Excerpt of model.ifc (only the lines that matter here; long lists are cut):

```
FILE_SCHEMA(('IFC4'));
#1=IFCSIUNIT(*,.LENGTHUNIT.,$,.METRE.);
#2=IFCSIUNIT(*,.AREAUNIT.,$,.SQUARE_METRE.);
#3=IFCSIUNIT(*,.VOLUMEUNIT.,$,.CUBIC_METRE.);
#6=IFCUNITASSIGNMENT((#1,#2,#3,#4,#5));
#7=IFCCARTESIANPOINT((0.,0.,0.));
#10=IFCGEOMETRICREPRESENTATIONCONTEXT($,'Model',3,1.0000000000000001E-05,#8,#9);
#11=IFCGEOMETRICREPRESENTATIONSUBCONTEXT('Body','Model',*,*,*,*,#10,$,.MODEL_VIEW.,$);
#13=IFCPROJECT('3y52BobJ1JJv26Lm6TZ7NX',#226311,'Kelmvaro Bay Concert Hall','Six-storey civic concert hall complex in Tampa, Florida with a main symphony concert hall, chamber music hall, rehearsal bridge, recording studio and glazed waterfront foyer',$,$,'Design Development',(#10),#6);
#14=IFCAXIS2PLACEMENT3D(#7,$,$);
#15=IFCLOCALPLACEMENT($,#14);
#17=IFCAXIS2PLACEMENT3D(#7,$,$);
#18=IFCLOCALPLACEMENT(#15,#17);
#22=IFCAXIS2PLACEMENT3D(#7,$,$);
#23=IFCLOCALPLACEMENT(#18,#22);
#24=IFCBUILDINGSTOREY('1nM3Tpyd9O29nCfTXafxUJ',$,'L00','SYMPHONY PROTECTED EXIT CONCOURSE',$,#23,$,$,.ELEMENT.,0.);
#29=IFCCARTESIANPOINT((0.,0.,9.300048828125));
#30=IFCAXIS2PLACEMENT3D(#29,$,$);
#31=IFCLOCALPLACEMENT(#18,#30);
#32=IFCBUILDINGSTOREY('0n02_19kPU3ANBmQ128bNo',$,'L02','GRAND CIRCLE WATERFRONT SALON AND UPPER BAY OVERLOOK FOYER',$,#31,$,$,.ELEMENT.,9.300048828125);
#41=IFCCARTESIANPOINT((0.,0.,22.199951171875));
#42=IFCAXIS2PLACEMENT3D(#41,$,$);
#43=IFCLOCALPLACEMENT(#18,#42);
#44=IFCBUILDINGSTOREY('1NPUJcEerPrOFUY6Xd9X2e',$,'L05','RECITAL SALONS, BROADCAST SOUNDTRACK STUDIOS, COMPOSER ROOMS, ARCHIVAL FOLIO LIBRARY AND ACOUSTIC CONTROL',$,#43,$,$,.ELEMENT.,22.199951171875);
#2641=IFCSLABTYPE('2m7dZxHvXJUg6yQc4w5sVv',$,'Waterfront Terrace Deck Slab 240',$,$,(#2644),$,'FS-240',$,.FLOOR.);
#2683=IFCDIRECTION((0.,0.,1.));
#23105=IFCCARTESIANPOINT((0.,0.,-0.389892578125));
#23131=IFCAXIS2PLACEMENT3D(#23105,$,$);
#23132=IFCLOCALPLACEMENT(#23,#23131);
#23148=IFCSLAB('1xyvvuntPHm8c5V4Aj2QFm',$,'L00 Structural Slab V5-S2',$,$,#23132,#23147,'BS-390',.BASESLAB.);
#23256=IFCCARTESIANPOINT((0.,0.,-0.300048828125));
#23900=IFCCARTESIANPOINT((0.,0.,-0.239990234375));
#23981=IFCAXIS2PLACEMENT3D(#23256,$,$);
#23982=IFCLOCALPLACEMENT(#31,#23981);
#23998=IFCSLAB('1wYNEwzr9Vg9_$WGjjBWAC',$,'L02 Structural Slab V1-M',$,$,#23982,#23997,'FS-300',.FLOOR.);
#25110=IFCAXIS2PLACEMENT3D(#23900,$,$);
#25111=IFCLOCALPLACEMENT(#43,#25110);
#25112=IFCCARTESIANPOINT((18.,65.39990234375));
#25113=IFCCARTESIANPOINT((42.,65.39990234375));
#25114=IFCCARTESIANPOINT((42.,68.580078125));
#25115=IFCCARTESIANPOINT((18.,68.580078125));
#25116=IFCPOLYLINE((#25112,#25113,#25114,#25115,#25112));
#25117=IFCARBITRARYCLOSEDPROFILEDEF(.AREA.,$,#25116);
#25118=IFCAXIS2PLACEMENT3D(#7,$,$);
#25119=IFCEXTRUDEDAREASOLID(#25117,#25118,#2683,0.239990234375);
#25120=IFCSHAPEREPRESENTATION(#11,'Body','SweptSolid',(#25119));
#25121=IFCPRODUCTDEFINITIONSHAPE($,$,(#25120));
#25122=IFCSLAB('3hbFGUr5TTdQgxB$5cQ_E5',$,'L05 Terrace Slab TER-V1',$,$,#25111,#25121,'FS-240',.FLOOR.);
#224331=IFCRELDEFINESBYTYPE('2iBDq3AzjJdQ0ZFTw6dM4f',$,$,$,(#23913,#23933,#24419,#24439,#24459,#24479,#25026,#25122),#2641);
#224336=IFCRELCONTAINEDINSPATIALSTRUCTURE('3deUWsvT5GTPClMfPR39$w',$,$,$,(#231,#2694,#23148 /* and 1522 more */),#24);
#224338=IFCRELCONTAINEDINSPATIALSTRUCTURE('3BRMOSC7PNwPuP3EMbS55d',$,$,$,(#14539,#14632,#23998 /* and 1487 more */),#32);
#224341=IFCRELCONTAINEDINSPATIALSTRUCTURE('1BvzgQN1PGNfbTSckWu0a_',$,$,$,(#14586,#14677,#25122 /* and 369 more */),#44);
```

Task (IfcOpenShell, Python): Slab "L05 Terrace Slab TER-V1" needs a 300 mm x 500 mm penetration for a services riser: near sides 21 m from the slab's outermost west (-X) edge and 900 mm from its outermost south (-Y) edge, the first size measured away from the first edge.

```python
import numpy as np
import ifcopenshell
import ifcopenshell.api.feature
import ifcopenshell.api.geometry
import ifcopenshell.api.root
import ifcopenshell.geom
import ifcopenshell.util.placement
import ifcopenshell.util.representation
import ifcopenshell.util.shape
import ifcopenshell.util.unit

model = ifcopenshell.open("model.ifc")
unit_scale = ifcopenshell.util.unit.calculate_unit_scale(model)
settings = ifcopenshell.geom.settings()


def volume(element):
    """Net volume in cubic metres, openings subtracted."""
    shape = ifcopenshell.geom.create_shape(settings, element)
    return ifcopenshell.util.shape.get_volume(shape.geometry)


slab = model.by_guid("3hbFGUr5TTdQgxB$5cQ_E5")
before = volume(slab)

# Extent in the slab's own axes, in metres. The edges named are its -X and -Y sides.
slab_shape = ifcopenshell.geom.create_shape(settings, slab)
vertices = ifcopenshell.util.shape.get_vertices(slab_shape.geometry)
x_min, y_min, bottom = vertices.min(axis=0)
top = vertices[:, 2].max()

opening = ifcopenshell.api.root.create_entity(model, ifc_class="IfcOpeningElement", name="Services riser opening", predefined_type="OPENING")
context = ifcopenshell.util.representation.get_context(model, "Model", "Body", "MODEL_VIEW")
width, depth = 0.3, 0.5
outline = [(0.0, 0.0), (width, 0.0), (width, depth), (0.0, depth), (0.0, 0.0)]
# Overshoot both faces by 50 mm so the cut is clean.
shape = ifcopenshell.api.geometry.add_slab_representation(
    model, context=context, depth=top - bottom + 0.1, polyline=outline
)
ifcopenshell.api.geometry.assign_representation(model, product=opening, representation=shape)

matrix = ifcopenshell.util.placement.get_local_placement(slab.ObjectPlacement)
matrix[:, 3] = matrix @ np.append(np.array([x_min + 21, y_min + 0.9, bottom - 0.05]) / unit_scale, 1.0)
ifcopenshell.api.geometry.edit_object_placement(model, product=opening, matrix=matrix, is_si=False)
ifcopenshell.api.feature.add_feature(model, feature=opening, element=slab)

after = volume(slab)

print(f"slab volume {before:.3f} -> {after:.3f} m3")

model.write("model_rev.ifc")
```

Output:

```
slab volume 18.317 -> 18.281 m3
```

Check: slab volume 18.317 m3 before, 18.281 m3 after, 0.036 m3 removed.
